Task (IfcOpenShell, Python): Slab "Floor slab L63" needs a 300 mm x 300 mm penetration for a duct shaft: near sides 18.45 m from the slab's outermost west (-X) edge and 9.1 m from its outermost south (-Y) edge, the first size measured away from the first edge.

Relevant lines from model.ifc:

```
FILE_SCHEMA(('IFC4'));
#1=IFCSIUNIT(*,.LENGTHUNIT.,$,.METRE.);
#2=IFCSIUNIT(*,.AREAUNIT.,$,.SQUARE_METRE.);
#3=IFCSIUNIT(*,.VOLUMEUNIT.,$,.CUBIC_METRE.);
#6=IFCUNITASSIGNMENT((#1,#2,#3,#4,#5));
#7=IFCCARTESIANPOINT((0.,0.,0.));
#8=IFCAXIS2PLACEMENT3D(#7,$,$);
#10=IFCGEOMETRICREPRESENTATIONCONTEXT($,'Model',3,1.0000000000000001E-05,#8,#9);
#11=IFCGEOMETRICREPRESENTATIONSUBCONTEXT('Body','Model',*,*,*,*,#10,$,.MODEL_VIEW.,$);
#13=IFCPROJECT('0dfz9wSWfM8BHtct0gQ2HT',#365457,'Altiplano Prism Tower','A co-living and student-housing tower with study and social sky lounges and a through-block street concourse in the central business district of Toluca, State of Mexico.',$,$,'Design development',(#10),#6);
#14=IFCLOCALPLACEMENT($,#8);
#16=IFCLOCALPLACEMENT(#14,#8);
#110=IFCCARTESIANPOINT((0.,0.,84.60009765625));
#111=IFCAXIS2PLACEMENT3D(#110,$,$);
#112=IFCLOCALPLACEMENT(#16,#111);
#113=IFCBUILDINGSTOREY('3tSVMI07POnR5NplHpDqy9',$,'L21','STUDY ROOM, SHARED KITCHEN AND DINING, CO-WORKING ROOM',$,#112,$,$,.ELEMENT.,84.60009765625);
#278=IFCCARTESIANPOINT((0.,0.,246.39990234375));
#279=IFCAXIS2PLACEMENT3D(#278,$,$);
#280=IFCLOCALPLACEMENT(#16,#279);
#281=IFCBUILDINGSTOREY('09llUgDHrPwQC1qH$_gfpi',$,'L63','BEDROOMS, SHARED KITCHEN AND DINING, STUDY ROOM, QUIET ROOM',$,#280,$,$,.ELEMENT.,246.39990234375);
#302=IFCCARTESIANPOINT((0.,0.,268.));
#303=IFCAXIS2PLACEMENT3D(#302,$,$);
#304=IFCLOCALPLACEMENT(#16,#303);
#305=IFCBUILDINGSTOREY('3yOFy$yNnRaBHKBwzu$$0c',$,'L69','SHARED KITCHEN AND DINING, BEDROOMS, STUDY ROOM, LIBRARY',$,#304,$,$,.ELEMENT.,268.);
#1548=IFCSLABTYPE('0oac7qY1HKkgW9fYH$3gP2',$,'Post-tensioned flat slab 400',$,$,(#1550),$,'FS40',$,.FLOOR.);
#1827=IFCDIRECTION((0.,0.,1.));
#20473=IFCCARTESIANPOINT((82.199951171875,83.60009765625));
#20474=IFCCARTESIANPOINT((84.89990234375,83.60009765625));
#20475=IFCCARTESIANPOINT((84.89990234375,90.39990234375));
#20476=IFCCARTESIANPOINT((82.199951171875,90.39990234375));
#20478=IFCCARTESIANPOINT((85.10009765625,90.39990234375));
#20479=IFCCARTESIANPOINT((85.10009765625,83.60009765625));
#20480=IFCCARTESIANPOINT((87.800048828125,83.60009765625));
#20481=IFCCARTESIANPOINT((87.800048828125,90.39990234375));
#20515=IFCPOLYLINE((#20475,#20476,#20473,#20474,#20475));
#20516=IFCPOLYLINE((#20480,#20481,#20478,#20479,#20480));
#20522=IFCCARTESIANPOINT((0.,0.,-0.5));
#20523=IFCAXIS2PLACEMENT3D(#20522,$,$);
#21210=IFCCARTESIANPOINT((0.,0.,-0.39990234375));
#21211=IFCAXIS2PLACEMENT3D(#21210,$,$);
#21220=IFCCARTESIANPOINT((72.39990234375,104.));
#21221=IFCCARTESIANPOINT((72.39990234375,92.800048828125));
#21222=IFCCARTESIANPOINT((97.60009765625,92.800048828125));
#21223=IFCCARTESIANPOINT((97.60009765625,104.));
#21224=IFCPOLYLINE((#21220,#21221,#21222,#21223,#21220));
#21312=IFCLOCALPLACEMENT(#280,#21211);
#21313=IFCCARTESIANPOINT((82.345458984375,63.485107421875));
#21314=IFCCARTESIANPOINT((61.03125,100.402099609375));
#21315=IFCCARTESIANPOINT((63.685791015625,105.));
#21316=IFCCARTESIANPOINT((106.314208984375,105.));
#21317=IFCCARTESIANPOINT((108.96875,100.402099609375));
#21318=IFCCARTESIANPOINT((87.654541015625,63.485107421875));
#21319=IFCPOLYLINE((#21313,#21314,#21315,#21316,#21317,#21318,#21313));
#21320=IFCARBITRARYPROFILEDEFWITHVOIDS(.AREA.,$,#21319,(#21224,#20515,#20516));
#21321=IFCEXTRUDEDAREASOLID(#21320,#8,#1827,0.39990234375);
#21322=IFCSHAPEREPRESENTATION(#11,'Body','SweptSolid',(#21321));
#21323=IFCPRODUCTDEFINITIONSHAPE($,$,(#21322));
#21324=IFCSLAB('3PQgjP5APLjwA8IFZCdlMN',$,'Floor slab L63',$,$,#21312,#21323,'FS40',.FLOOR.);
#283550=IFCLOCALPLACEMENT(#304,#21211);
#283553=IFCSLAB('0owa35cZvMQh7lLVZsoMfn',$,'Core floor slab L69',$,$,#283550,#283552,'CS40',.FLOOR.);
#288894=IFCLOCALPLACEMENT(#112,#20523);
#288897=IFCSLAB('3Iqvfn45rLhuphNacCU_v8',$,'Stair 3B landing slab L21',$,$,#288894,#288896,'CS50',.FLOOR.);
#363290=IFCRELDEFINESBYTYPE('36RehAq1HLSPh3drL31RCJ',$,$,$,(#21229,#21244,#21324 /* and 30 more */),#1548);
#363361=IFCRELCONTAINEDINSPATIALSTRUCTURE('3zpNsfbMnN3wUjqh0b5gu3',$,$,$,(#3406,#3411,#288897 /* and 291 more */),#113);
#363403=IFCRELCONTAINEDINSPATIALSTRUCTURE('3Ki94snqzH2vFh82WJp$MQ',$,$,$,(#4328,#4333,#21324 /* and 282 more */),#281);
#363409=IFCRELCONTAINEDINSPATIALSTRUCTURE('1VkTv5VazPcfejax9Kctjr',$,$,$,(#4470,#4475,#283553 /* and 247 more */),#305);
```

```python
import numpy as np
import ifcopenshell
import ifcopenshell.api.feature
import ifcopenshell.api.geometry
import ifcopenshell.api.root
import ifcopenshell.geom
import ifcopenshell.util.placement
import ifcopenshell.util.representation
import ifcopenshell.util.shape
import ifcopenshell.util.unit

model = ifcopenshell.open("model.ifc")
unit_scale = ifcopenshell.util.unit.calculate_unit_scale(model)
settings = ifcopenshell.geom.settings()


def volume(element):
    """Net volume in cubic metres, openings subtracted."""
    shape = ifcopenshell.geom.create_shape(settings, element)
    return ifcopenshell.util.shape.get_volume(shape.geometry)


slab = model.by_guid("3PQgjP5APLjwA8IFZCdlMN")
before = volume(slab)

# Extent in the slab's own axes, in metres. The edges named are its -X and -Y sides.
slab_shape = ifcopenshell.geom.create_shape(settings, slab)
vertices = ifcopenshell.util.shape.get_vertices(slab_shape.geometry)
x_min, y_min, bottom = vertices.min(axis=0)
top = vertices[:, 2].max()

opening = ifcopenshell.api.root.create_entity(model, ifc_class="IfcOpeningElement", name="Duct shaft opening", predefined_type="OPENING")
context = ifcopenshell.util.representation.get_context(model, "Model", "Body", "MODEL_VIEW")
width, depth = 0.3, 0.3
outline = [(0.0, 0.0), (width, 0.0), (width, depth), (0.0, depth), (0.0, 0.0)]
# Overshoot both faces by 50 mm so the cut is clean.
shape = ifcopenshell.api.geometry.add_slab_representation(
    model, context=context, depth=top - bottom + 0.1, polyline=outline
)
ifcopenshell.api.geometry.assign_representation(model, product=opening, representation=shape)

matrix = ifcopenshell.util.placement.get_local_placement(slab.ObjectPlacement)
matrix[:, 3] = matrix @ np.append(np.array([x_min + 18.45, y_min + 9.1, bottom - 0.05]) / unit_scale, 1.0)
ifcopenshell.api.geometry.edit_object_placement(model, product=opening, matrix=matrix, is_si=False)
ifcopenshell.api.feature.add_feature(model, feature=opening, element=slab)

after = volume(slab)

print(f"slab volume {before:.3f} -> {after:.3f} m3")

model.write("model_edited.ifc")
```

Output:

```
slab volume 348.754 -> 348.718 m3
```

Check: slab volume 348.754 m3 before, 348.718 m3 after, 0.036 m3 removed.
